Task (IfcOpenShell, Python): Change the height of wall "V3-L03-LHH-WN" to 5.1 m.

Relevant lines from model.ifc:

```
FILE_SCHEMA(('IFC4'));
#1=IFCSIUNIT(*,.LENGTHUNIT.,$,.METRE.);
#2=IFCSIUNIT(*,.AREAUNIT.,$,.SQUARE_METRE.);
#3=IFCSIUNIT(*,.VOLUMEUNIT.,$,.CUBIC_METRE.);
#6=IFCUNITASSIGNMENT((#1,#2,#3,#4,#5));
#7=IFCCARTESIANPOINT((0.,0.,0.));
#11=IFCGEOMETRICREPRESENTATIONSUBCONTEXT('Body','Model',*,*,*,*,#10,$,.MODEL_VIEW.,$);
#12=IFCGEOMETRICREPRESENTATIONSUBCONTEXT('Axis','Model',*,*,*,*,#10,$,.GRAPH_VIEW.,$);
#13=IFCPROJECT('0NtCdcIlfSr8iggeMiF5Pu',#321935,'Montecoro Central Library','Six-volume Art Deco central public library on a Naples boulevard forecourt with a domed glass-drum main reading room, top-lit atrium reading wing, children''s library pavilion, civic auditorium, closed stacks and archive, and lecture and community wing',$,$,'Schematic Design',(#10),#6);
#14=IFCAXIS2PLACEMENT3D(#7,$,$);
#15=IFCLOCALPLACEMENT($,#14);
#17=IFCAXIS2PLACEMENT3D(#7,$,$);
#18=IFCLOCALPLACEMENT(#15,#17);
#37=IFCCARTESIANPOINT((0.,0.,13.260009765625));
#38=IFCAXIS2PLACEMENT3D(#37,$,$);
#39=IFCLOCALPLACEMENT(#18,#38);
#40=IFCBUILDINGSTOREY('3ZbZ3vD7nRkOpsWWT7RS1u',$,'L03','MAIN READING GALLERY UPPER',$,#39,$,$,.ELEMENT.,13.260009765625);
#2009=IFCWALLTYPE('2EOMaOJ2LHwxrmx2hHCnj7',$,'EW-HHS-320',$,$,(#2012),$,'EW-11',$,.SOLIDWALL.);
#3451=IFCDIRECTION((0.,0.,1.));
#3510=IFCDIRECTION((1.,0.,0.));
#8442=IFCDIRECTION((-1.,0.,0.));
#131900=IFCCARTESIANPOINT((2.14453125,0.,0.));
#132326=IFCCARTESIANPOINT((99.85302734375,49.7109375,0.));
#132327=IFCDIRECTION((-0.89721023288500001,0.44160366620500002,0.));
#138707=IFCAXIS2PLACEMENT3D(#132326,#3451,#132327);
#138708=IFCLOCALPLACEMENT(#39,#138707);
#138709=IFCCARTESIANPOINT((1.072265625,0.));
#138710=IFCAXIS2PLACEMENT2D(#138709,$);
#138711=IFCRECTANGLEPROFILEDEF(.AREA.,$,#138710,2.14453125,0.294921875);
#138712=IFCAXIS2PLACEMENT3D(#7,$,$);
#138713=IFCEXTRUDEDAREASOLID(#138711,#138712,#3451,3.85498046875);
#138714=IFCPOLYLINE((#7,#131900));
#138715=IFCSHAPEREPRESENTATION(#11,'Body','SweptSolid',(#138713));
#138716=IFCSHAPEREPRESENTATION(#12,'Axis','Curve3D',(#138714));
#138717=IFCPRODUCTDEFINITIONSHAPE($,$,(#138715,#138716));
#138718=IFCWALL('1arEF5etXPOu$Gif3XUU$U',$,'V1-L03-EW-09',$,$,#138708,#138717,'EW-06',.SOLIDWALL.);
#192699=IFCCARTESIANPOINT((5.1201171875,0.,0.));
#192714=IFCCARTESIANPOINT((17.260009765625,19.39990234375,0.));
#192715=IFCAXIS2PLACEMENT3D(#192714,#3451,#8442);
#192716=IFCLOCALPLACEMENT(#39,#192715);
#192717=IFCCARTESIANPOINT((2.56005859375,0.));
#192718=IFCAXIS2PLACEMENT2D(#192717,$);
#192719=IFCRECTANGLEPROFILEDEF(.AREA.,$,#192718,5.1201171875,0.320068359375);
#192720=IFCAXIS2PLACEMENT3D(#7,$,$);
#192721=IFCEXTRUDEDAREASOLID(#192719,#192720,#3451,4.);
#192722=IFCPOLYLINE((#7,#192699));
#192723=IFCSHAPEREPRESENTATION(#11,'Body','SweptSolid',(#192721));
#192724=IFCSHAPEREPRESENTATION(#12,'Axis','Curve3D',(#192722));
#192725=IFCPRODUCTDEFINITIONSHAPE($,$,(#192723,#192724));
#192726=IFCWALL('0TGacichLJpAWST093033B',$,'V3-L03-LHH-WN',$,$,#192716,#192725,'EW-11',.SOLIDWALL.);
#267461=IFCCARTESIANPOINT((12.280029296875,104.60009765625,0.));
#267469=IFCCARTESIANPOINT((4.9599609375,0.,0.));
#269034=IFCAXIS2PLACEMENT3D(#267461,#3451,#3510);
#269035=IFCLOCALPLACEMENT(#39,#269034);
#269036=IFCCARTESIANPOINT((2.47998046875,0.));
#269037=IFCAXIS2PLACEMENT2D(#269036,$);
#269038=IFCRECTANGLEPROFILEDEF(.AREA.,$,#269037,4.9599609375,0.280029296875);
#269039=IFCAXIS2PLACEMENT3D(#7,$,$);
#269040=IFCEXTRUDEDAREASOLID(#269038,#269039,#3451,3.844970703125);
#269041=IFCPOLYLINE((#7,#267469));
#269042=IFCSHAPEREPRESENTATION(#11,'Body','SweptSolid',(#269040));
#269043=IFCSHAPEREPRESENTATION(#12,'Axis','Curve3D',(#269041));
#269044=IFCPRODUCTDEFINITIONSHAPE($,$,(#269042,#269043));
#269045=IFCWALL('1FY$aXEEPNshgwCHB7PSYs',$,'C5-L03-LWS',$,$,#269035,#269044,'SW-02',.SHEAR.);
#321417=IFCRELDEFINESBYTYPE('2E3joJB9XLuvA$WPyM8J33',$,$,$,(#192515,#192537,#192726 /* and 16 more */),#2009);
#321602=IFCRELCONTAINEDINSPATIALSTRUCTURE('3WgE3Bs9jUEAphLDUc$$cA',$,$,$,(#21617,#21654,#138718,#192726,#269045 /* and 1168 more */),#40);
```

```python
import ifcopenshell
import ifcopenshell.geom
import ifcopenshell.util.representation
import ifcopenshell.util.shape

model = ifcopenshell.open("model.ifc")
settings = ifcopenshell.geom.settings()


def volume(element):
    """Net volume in cubic metres, openings subtracted."""
    shape = ifcopenshell.geom.create_shape(settings, element)
    return ifcopenshell.util.shape.get_volume(shape.geometry)


wall = model.by_guid("0TGacichLJpAWST093033B")
before = volume(wall)

body = ifcopenshell.util.representation.get_representation(wall, "Model", "Body")
solid = body.Items[0]
old_height = solid.Depth
solid.Depth = 5.1
after = volume(wall)

print(f"height {old_height:g} -> {solid.Depth:g}, volume {before:.3f} -> {after:.3f} m3")

model.write("model_rev.ifc")
```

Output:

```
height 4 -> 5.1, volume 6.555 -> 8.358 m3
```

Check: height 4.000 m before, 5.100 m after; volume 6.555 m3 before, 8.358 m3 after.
